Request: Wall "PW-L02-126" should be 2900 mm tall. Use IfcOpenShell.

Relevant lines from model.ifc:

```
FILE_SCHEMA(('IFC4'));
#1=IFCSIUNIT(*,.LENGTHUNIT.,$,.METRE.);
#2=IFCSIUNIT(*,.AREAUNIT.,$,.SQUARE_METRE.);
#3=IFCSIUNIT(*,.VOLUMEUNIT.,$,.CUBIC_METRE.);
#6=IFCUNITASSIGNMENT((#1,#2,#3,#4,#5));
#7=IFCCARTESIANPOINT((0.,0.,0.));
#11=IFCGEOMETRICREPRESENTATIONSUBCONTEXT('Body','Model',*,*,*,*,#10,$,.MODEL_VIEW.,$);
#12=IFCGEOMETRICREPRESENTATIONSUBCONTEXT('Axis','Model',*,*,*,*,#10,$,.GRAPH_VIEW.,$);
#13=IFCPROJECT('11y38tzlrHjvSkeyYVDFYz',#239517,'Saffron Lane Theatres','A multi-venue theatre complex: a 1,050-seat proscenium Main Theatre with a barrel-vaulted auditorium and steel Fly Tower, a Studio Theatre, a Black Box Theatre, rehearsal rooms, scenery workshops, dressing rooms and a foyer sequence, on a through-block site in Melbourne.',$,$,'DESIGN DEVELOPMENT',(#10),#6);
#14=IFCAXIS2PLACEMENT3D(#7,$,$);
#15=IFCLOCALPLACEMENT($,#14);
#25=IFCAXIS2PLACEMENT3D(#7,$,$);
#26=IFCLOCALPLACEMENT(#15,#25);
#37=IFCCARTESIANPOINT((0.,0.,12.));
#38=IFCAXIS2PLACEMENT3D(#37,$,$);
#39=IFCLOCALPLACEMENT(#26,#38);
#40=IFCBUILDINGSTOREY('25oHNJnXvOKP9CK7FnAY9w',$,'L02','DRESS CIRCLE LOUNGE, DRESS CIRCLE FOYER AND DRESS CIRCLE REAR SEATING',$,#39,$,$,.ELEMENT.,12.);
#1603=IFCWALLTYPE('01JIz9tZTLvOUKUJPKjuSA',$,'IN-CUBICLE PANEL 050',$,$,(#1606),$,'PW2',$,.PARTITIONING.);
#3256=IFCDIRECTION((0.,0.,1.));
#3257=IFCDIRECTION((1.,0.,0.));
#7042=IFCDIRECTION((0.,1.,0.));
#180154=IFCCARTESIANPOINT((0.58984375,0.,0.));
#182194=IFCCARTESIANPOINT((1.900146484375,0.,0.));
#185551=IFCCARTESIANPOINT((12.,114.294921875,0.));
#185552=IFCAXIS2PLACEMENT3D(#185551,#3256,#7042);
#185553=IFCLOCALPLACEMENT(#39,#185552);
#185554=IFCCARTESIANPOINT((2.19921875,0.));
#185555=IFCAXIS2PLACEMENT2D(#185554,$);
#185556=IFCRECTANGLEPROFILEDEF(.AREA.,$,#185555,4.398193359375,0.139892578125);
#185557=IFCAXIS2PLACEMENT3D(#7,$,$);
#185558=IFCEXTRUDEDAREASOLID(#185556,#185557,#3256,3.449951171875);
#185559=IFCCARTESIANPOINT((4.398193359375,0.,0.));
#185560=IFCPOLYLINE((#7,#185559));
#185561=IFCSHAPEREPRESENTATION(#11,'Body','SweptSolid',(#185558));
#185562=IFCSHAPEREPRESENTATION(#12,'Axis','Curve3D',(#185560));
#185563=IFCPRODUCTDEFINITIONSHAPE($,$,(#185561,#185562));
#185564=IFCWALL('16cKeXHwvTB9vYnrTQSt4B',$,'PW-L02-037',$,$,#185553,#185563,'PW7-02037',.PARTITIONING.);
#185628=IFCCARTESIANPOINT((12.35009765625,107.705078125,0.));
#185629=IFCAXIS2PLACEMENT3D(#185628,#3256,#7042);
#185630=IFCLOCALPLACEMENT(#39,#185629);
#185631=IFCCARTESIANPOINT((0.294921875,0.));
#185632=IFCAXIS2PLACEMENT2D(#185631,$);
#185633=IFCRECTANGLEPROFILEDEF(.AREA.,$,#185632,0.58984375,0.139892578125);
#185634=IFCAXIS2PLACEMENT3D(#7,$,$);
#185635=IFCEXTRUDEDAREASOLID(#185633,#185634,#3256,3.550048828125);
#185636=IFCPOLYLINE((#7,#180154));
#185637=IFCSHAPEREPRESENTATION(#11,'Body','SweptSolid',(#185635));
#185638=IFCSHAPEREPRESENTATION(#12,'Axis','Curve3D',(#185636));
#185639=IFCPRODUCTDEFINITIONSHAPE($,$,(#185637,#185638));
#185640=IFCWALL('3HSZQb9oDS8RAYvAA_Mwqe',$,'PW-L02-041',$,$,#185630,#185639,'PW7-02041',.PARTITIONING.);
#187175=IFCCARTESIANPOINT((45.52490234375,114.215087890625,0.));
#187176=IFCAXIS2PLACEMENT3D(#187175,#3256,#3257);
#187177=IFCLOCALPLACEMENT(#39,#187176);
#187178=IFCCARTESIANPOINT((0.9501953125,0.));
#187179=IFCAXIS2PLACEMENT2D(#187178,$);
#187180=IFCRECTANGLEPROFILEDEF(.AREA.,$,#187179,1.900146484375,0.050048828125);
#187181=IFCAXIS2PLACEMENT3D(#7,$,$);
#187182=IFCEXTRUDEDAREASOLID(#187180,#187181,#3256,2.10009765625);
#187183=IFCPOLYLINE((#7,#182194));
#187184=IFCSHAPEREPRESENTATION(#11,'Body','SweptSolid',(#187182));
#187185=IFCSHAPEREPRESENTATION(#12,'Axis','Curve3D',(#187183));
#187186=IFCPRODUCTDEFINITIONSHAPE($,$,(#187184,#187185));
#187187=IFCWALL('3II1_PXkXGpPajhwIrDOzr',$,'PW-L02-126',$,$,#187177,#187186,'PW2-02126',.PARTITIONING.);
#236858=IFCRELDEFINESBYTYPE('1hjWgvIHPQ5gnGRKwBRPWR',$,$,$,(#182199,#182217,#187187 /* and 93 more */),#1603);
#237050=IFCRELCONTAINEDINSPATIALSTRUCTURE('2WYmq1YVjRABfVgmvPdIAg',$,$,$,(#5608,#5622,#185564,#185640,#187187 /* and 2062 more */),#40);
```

```python
import ifcopenshell
import ifcopenshell.geom
import ifcopenshell.util.representation
import ifcopenshell.util.shape
import ifcopenshell.util.unit

model = ifcopenshell.open("model.ifc")
unit_scale = ifcopenshell.util.unit.calculate_unit_scale(model)
settings = ifcopenshell.geom.settings()


def volume(element):
    """Net volume in cubic metres, openings subtracted."""
    shape = ifcopenshell.geom.create_shape(settings, element)
    return ifcopenshell.util.shape.get_volume(shape.geometry)


wall = model.by_guid("3II1_PXkXGpPajhwIrDOzr")
before = volume(wall)

body = ifcopenshell.util.representation.get_representation(wall, "Model", "Body")
solid = body.Items[0]
old_height = solid.Depth
solid.Depth = 2.9 / unit_scale
after = volume(wall)

print(f"height {old_height:g} -> {solid.Depth:g}, volume {before:.3f} -> {after:.3f} m3")

model.write("model_rev.ifc")
```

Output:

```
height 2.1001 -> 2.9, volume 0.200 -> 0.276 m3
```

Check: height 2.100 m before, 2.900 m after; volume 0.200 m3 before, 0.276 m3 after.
